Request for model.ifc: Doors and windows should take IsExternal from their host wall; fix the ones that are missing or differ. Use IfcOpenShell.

First a look at what the model holds.

```python
import ifcopenshell
import ifcopenshell.util.element

model = ifcopenshell.open("model.ifc")
print(model.schema)
seen = {}
for e in model.by_type("IfcDoor") + model.by_type("IfcWindow"):
    if not e.FillsVoids:
        continue
    host = e.FillsVoids[0].RelatingOpeningElement.VoidsElements[0].RelatingBuildingElement
    own = ifcopenshell.util.element.get_pset(e, f"Pset_{e.is_a()[3:].removesuffix('StandardCase')}Common", "IsExternal")
    wall = ifcopenshell.util.element.get_pset(host, "Pset_WallCommon", "IsExternal")
    seen[e.is_a(), own, wall] = seen.get((e.is_a(), own, wall), 0) + 1
for (cls, own, wall), count in sorted(seen.items(), key=str):
    print(count, cls, "IsExternal:", own, "| host wall:", wall)
```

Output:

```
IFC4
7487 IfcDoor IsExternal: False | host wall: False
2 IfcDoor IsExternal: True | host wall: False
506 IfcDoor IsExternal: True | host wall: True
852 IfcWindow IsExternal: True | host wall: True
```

```python
import ifcopenshell
import ifcopenshell.api.pset
import ifcopenshell.util.element

model = ifcopenshell.open("model.ifc")

count = 0
for ifc_class, pset_name in (("IfcDoor", "Pset_DoorCommon"), ("IfcWindow", "Pset_WindowCommon")):
    for e in model.by_type(ifc_class):
        if not e.FillsVoids:
            continue
        host = e.FillsVoids[0].RelatingOpeningElement.VoidsElements[0].RelatingBuildingElement
        external = ifcopenshell.util.element.get_pset(host, "Pset_WallCommon", "IsExternal")
        if external is None or ifcopenshell.util.element.get_pset(e, pset_name, "IsExternal") == external:
            continue
        found = ifcopenshell.util.element.get_pset(e, pset_name, should_inherit=False)
        if found:
            pset = model.by_id(found["id"])
            if len(ifcopenshell.util.element.get_elements_by_pset(pset)) > 1:
                pset = ifcopenshell.api.pset.unshare_pset(model, products=[e], pset=pset)[0]
        else:
            pset = ifcopenshell.api.pset.add_pset(model, product=e, name=pset_name)
        ifcopenshell.api.pset.edit_pset(model, pset=pset, properties={"IsExternal": external})
        count += 1

print(count, "updated")

model.write("model_v2.ifc")
```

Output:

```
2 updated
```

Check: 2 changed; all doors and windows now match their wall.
